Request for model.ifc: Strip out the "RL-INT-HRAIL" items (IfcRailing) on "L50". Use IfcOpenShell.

First a look at what the model holds.

```python
import ifcopenshell
import ifcopenshell.util.element

model = ifcopenshell.open("model.ifc")
print(model.schema)
storey = next(s for s in model.by_type("IfcBuildingStorey") if s.Name == "L50")
railings = [e for e in ifcopenshell.util.element.get_decomposition(storey) if e.is_a("IfcRailing")]
seen = {}
for e in railings:
    element_type = ifcopenshell.util.element.get_type(e)
    name = element_type.Name if element_type not in (None, e) else None
    seen[name] = seen.get(name, 0) + 1
for name, count in sorted(seen.items(), key=str):
    print(count, "x", name)
```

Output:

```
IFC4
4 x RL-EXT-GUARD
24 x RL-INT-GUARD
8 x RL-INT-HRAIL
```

```python
import ifcopenshell
import ifcopenshell.api.root
import ifcopenshell.util.element

model = ifcopenshell.open("model.ifc")

storey = next(s for s in model.by_type("IfcBuildingStorey") if s.Name == "L50")
railings = [e for e in ifcopenshell.util.element.get_decomposition(storey) if e.is_a("IfcRailing")]
targets = [e for e in railings if (t := ifcopenshell.util.element.get_type(e)) not in (None, e) and t.Name == "RL-INT-HRAIL"]

for e in targets:
    ifcopenshell.api.root.remove_product(model, product=e)
print(len(targets), "removed")

model.write("model_edited.ifc")
```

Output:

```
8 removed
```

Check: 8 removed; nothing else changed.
